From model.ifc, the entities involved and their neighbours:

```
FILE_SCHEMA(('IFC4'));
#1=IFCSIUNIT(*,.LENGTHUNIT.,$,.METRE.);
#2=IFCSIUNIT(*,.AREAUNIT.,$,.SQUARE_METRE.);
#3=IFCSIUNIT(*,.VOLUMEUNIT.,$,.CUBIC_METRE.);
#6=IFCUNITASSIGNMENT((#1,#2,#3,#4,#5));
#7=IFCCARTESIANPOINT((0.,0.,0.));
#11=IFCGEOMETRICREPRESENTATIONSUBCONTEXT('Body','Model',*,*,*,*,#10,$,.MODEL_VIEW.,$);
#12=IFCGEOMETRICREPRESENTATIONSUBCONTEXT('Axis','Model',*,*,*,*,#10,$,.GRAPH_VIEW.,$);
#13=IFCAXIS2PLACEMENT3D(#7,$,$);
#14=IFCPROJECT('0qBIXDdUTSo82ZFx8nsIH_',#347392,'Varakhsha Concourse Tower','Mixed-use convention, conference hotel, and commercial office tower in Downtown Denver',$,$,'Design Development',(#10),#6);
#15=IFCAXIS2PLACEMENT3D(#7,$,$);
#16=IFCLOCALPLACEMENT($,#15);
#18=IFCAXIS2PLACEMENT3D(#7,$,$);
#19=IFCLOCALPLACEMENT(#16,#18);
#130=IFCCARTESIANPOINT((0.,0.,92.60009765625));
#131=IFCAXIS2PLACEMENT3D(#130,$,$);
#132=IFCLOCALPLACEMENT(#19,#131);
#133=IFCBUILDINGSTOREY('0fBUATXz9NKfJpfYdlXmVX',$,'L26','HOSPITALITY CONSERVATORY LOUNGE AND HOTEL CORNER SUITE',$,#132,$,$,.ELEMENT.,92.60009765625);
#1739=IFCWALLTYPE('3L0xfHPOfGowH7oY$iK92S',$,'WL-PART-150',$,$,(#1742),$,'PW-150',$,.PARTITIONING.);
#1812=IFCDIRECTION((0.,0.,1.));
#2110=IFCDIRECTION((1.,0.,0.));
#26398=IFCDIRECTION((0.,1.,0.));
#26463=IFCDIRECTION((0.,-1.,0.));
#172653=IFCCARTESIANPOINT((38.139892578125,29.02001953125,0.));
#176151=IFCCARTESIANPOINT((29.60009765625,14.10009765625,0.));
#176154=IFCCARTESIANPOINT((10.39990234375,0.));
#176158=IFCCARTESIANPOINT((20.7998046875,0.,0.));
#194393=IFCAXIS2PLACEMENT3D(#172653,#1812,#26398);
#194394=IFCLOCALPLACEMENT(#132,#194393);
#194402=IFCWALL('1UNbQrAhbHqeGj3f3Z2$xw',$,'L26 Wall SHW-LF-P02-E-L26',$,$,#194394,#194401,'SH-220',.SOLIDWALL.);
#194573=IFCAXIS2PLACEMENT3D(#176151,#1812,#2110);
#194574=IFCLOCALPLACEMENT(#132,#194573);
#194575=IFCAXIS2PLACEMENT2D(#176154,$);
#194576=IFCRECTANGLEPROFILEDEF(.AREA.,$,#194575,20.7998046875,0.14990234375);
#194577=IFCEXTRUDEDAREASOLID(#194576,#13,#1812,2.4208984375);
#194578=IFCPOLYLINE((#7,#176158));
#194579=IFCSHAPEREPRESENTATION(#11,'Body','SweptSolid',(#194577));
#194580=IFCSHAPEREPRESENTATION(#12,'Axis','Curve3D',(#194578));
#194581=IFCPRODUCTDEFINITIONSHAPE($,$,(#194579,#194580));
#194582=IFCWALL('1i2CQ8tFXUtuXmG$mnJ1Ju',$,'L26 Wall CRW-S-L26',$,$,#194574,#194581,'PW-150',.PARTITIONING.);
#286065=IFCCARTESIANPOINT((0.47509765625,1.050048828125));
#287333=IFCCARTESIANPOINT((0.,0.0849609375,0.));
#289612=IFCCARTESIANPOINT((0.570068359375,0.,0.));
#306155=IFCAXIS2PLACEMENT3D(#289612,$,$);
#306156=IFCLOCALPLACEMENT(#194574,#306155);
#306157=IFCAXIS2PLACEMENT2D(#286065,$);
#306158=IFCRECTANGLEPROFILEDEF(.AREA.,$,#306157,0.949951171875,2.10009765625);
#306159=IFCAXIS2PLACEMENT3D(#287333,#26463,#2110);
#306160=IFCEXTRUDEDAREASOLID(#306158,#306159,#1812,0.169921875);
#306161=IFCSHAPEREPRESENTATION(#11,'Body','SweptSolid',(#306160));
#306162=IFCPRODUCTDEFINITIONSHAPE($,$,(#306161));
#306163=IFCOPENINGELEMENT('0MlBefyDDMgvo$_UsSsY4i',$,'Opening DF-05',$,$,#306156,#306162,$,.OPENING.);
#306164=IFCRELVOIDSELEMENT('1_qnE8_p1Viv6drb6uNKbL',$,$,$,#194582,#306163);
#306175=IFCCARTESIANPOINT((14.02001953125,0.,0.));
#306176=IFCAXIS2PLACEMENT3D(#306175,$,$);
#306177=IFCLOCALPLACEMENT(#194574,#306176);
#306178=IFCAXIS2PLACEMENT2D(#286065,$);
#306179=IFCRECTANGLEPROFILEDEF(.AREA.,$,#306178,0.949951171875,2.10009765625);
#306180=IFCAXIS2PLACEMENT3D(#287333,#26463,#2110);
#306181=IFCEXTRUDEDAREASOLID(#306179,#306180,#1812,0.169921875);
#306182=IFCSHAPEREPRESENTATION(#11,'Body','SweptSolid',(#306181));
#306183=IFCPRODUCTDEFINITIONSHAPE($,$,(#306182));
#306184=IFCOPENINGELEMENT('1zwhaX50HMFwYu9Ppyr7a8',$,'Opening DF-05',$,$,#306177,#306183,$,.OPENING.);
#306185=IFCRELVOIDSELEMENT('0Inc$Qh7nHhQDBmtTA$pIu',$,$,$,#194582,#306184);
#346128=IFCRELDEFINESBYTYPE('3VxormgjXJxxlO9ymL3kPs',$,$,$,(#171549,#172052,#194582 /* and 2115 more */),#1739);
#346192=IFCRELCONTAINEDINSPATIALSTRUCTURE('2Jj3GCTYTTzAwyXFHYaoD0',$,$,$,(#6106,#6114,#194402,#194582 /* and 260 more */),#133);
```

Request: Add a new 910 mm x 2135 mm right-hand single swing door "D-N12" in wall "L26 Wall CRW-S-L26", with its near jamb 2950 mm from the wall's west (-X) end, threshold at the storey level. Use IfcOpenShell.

```python
import numpy as np
import ifcopenshell
import ifcopenshell.api.feature
import ifcopenshell.api.geometry
import ifcopenshell.api.root
import ifcopenshell.api.spatial
import ifcopenshell.geom
import ifcopenshell.util.element
import ifcopenshell.util.placement
import ifcopenshell.util.representation
import ifcopenshell.util.shape
import ifcopenshell.util.unit

model = ifcopenshell.open("model.ifc")
unit_scale = ifcopenshell.util.unit.calculate_unit_scale(model)
settings = ifcopenshell.geom.settings()


def volume(element):
    """Net volume in cubic metres, openings subtracted."""
    shape = ifcopenshell.geom.create_shape(settings, element)
    return ifcopenshell.util.shape.get_volume(shape.geometry)


wall = model.by_id(194582)
storey = ifcopenshell.util.element.get_container(wall, ifc_class="IfcBuildingStorey")
context = ifcopenshell.util.representation.get_context(model, "Model", "Body", "MODEL_VIEW")
before = volume(wall)

width, height, from_end, sill = 0.91, 2.135, 2.95, 0.0  # metres

# The wall runs along its own X axis, and the end named is its -X end.
wall_shape = ifcopenshell.geom.create_shape(settings, wall)
x, y, z = ifcopenshell.util.shape.get_vertices(wall_shape.geometry).T
start = x.min() + from_end
face, thickness = float(y.min()), float(y.max() - y.min())
wall_matrix = ifcopenshell.util.placement.get_local_placement(wall.ObjectPlacement)
level = ifcopenshell.util.placement.get_local_placement(storey.ObjectPlacement)[2, 3]


def in_wall(x, y):
    """Placement at x, y metres in the wall's axes, at sill height."""
    matrix = wall_matrix.copy()
    matrix[:, 3] = wall_matrix @ np.array([x / unit_scale, y / unit_scale, 0.0, 1.0])
    matrix[2, 3] = level + sill / unit_scale
    return matrix


# Opening: a box that overshoots both wall faces by 50 mm.
opening = ifcopenshell.api.root.create_entity(model, ifc_class="IfcOpeningElement", predefined_type="OPENING")
box = ifcopenshell.api.geometry.add_wall_representation(
    model, context=context, length=width, height=height, thickness=thickness + 0.1
)
ifcopenshell.api.geometry.assign_representation(model, product=opening, representation=box)
ifcopenshell.api.geometry.edit_object_placement(model, product=opening, matrix=in_wall(start, face - 0.05), is_si=False)
ifcopenshell.api.feature.add_feature(model, feature=opening, element=wall)

door = ifcopenshell.api.root.create_entity(model, ifc_class="IfcDoor", name="D-N12", predefined_type="DOOR")
door.OverallWidth, door.OverallHeight = width / unit_scale, height / unit_scale
door.OperationType = "SINGLE_SWING_RIGHT"
body = ifcopenshell.api.geometry.add_door_representation(
    model,
    context=context,
    overall_width=door.OverallWidth,
    overall_height=door.OverallHeight,
    operation_type="SINGLE_SWING_RIGHT",
    lining_properties={"LiningDepth": thickness / unit_scale, "ThresholdDepth": thickness / unit_scale},
)
ifcopenshell.api.geometry.assign_representation(model, product=door, representation=body)
ifcopenshell.api.spatial.assign_container(model, products=[door], relating_structure=storey)
ifcopenshell.api.feature.add_filling(model, opening=opening, element=door)

# The lining spans the wall, so the door starts at the wall face.
ifcopenshell.api.geometry.edit_object_placement(model, product=door, matrix=in_wall(start, face), is_si=False)

after = volume(wall)

print(f"wall volume {before:.3f} -> {after:.3f} m3")

model.write("model_v2.ifc")
```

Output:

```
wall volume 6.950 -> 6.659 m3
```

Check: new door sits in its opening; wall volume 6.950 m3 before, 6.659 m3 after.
